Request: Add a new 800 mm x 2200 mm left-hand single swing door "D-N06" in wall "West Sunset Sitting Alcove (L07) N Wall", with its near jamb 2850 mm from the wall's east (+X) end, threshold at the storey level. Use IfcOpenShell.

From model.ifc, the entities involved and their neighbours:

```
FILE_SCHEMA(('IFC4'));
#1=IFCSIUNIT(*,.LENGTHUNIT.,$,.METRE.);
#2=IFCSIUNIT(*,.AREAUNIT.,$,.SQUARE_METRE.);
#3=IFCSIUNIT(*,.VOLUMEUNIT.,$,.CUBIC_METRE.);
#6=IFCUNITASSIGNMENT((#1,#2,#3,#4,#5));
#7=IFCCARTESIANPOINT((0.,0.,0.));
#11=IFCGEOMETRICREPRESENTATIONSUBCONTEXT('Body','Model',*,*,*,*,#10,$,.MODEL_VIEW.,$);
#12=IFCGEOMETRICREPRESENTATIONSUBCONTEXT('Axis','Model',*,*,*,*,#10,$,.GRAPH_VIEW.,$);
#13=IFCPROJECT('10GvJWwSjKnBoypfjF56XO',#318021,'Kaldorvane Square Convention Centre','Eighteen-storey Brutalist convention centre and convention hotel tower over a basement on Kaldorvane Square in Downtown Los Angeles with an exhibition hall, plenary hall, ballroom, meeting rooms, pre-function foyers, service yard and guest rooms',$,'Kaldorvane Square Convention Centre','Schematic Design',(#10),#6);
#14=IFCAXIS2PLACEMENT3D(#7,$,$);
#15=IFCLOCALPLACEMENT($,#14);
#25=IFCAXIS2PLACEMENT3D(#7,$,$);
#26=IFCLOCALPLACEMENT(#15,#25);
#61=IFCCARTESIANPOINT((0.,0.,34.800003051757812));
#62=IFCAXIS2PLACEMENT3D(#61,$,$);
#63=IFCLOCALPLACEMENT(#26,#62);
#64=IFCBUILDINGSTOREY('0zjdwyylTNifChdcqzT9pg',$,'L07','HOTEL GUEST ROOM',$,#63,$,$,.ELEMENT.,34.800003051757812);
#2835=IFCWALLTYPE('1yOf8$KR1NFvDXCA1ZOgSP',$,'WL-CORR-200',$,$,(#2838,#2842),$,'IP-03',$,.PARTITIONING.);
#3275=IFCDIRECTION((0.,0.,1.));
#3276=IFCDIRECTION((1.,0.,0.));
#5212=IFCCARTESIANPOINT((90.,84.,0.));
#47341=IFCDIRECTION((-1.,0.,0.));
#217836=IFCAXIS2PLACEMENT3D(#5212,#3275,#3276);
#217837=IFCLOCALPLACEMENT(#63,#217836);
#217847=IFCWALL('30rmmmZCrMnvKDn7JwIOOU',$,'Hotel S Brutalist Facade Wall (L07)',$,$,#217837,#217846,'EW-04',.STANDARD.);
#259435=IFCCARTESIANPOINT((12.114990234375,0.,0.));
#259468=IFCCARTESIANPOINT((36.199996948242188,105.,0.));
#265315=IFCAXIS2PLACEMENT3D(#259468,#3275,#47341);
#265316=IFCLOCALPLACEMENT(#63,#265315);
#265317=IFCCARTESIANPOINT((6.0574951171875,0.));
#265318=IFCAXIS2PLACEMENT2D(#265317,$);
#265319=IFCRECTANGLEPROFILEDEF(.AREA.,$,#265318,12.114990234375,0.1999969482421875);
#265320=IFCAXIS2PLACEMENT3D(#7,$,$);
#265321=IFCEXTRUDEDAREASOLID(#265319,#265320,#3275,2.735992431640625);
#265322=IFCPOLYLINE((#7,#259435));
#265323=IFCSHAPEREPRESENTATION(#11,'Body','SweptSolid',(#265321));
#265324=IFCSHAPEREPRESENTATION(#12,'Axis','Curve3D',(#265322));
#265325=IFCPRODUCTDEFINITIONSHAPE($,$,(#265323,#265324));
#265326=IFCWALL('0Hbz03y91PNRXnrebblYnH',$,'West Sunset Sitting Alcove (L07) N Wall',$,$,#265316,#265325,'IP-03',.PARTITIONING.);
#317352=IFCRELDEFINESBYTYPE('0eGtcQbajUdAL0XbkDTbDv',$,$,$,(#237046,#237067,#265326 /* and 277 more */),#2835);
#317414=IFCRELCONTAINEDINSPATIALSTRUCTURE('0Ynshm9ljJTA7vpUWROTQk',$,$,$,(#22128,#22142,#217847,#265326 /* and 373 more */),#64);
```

```python
import numpy as np
import ifcopenshell
import ifcopenshell.api.feature
import ifcopenshell.api.geometry
import ifcopenshell.api.root
import ifcopenshell.api.spatial
import ifcopenshell.geom
import ifcopenshell.util.element
import ifcopenshell.util.placement
import ifcopenshell.util.representation
import ifcopenshell.util.shape
import ifcopenshell.util.unit

model = ifcopenshell.open("model.ifc")
unit_scale = ifcopenshell.util.unit.calculate_unit_scale(model)
settings = ifcopenshell.geom.settings()


def volume(element):
    """Net volume in cubic metres, openings subtracted."""
    shape = ifcopenshell.geom.create_shape(settings, element)
    return ifcopenshell.util.shape.get_volume(shape.geometry)


wall = model.by_id(265326)
storey = ifcopenshell.util.element.get_container(wall, ifc_class="IfcBuildingStorey")
context = ifcopenshell.util.representation.get_context(model, "Model", "Body", "MODEL_VIEW")
before = volume(wall)

width, height, from_end, sill = 0.8, 2.2, 2.85, 0.0  # metres

# The wall runs along its own X axis, and the end named is its -X end.
wall_shape = ifcopenshell.geom.create_shape(settings, wall)
x, y, z = ifcopenshell.util.shape.get_vertices(wall_shape.geometry).T
start = x.min() + from_end
face, thickness = float(y.min()), float(y.max() - y.min())
wall_matrix = ifcopenshell.util.placement.get_local_placement(wall.ObjectPlacement)
level = ifcopenshell.util.placement.get_local_placement(storey.ObjectPlacement)[2, 3]


def in_wall(x, y):
    """Placement at x, y metres in the wall's axes, at sill height."""
    matrix = wall_matrix.copy()
    matrix[:, 3] = wall_matrix @ np.array([x / unit_scale, y / unit_scale, 0.0, 1.0])
    matrix[2, 3] = level + sill / unit_scale
    return matrix


# Opening: a box that overshoots both wall faces by 50 mm.
opening = ifcopenshell.api.root.create_entity(model, ifc_class="IfcOpeningElement", predefined_type="OPENING")
box = ifcopenshell.api.geometry.add_wall_representation(
    model, context=context, length=width, height=height, thickness=thickness + 0.1
)
ifcopenshell.api.geometry.assign_representation(model, product=opening, representation=box)
ifcopenshell.api.geometry.edit_object_placement(model, product=opening, matrix=in_wall(start, face - 0.05), is_si=False)
ifcopenshell.api.feature.add_feature(model, feature=opening, element=wall)

door = ifcopenshell.api.root.create_entity(model, ifc_class="IfcDoor", name="D-N06", predefined_type="DOOR")
door.OverallWidth, door.OverallHeight = width / unit_scale, height / unit_scale
door.OperationType = "SINGLE_SWING_LEFT"
body = ifcopenshell.api.geometry.add_door_representation(
    model,
    context=context,
    overall_width=door.OverallWidth,
    overall_height=door.OverallHeight,
    operation_type="SINGLE_SWING_LEFT",
    lining_properties={"LiningDepth": thickness / unit_scale, "ThresholdDepth": thickness / unit_scale},
)
ifcopenshell.api.geometry.assign_representation(model, product=door, representation=body)
ifcopenshell.api.spatial.assign_container(model, products=[door], relating_structure=storey)
ifcopenshell.api.feature.add_filling(model, opening=opening, element=door)

# The lining spans the wall, so the door starts at the wall face.
ifcopenshell.api.geometry.edit_object_placement(model, product=door, matrix=in_wall(start, face), is_si=False)

after = volume(wall)

print(f"wall volume {before:.3f} -> {after:.3f} m3")

model.write("model_updated.ifc")
```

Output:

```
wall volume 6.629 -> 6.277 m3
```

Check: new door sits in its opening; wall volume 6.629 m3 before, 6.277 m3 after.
